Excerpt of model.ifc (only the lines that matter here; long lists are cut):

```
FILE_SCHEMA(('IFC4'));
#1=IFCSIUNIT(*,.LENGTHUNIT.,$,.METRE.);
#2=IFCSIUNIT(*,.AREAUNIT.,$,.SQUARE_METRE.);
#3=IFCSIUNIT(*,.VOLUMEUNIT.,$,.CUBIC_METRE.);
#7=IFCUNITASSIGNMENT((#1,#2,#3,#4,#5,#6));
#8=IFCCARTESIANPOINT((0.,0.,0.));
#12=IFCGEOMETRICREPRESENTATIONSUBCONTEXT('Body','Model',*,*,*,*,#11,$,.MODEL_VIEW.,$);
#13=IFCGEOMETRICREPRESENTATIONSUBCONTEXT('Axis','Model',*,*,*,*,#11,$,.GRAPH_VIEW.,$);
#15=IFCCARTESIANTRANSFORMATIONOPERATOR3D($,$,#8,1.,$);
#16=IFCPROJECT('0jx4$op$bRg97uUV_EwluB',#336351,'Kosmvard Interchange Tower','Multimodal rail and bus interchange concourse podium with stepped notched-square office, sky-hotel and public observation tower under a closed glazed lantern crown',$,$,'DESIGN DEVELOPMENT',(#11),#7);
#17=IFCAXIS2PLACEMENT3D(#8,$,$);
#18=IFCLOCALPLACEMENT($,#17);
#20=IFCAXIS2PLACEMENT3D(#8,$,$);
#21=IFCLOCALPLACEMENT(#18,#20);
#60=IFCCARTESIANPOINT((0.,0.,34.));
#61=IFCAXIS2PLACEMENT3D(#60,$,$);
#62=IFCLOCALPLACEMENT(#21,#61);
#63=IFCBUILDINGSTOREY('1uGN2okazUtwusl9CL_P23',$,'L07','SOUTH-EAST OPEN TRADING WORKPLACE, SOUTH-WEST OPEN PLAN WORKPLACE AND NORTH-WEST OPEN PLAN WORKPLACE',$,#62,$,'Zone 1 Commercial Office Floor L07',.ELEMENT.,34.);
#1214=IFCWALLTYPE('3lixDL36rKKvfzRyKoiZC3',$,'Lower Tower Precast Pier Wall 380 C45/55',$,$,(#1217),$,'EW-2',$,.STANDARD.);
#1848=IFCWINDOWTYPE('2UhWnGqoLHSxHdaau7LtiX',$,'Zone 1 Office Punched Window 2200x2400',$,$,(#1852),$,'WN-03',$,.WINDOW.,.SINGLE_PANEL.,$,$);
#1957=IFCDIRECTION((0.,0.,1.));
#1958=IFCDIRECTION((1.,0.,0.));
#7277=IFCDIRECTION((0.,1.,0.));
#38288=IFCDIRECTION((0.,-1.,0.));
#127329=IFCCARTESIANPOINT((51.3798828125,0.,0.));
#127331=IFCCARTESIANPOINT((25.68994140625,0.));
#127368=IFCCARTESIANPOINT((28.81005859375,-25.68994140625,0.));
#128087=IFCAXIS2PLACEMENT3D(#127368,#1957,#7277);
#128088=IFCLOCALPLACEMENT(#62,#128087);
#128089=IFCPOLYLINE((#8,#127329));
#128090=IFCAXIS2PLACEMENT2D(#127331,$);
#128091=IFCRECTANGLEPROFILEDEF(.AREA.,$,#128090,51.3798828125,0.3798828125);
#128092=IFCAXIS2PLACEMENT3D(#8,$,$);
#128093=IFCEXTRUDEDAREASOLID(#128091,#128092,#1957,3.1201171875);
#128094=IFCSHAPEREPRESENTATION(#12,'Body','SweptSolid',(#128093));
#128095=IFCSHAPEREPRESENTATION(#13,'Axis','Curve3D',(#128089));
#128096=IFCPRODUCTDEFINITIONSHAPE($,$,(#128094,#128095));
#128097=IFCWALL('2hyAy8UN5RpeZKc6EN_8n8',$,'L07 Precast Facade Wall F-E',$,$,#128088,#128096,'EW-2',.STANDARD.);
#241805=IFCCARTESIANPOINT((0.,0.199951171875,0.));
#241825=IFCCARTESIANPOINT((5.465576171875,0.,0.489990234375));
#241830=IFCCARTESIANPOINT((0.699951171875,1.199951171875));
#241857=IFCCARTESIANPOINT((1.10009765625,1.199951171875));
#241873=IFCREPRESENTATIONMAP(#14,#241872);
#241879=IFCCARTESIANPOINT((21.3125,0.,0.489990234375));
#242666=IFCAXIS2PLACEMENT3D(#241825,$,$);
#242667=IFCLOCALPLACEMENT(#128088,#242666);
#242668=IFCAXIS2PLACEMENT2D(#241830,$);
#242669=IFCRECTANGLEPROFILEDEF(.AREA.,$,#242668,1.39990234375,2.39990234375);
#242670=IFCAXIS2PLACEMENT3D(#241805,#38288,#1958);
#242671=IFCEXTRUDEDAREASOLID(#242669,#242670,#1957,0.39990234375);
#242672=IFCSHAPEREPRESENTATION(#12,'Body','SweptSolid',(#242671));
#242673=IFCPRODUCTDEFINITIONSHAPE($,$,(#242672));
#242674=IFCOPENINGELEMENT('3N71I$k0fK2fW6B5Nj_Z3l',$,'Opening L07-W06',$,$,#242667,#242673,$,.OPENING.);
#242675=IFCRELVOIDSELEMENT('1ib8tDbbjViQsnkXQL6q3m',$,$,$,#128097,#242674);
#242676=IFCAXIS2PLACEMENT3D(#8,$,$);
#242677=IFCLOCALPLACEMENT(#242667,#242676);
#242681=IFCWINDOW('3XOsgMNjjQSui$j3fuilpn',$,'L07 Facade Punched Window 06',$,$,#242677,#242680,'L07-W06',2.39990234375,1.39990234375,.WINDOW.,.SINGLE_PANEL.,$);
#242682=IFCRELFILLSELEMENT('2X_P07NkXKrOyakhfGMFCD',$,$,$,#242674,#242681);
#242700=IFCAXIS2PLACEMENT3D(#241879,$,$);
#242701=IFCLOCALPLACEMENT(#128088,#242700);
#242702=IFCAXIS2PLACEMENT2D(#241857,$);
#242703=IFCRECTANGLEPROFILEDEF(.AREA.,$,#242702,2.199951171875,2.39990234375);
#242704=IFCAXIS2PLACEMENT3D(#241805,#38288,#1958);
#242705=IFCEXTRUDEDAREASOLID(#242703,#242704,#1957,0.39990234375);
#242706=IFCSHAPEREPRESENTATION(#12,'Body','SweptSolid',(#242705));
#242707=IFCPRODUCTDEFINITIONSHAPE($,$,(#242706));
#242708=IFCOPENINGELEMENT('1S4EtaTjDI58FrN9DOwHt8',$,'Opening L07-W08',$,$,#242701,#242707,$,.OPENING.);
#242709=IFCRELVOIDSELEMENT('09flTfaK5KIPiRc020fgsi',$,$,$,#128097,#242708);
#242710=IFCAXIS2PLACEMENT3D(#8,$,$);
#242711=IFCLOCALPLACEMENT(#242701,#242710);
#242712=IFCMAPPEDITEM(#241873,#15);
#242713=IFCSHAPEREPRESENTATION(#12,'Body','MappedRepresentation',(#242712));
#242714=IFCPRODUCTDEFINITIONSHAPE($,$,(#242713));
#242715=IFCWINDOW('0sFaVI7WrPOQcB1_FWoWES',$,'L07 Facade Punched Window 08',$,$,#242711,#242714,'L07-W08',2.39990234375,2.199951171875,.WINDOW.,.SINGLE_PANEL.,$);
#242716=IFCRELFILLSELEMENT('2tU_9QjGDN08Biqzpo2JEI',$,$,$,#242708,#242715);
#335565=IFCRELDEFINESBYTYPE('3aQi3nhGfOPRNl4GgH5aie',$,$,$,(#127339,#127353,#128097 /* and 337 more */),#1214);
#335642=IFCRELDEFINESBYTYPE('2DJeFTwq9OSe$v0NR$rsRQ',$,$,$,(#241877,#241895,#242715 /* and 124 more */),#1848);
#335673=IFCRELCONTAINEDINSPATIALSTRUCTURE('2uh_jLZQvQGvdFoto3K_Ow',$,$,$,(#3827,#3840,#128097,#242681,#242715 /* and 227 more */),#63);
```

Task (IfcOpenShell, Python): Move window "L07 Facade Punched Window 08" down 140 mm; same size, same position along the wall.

```python
import numpy as np
import ifcopenshell
import ifcopenshell.api.geometry
import ifcopenshell.util.placement
import ifcopenshell.util.unit

model = ifcopenshell.open("model.ifc")
unit_scale = ifcopenshell.util.unit.calculate_unit_scale(model)

window = model.by_guid("0sFaVI7WrPOQcB1_FWoWES")
opening = window.FillsVoids[0].RelatingOpeningElement
dz = -0.14

shift = np.array([0.0, 0.0, dz])
# The window is placed relative to its opening, so it follows when the opening moves.
matrix = ifcopenshell.util.placement.get_local_placement(opening.ObjectPlacement)
matrix[:3, 3] += shift
ifcopenshell.api.geometry.edit_object_placement(
    model, product=opening, matrix=matrix, is_si=False, should_transform_children=True
)

print(f"moved by {dz * unit_scale:+.3f} m")

model.write("model_v2.ifc")
```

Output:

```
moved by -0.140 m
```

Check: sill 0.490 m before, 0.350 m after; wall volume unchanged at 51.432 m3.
